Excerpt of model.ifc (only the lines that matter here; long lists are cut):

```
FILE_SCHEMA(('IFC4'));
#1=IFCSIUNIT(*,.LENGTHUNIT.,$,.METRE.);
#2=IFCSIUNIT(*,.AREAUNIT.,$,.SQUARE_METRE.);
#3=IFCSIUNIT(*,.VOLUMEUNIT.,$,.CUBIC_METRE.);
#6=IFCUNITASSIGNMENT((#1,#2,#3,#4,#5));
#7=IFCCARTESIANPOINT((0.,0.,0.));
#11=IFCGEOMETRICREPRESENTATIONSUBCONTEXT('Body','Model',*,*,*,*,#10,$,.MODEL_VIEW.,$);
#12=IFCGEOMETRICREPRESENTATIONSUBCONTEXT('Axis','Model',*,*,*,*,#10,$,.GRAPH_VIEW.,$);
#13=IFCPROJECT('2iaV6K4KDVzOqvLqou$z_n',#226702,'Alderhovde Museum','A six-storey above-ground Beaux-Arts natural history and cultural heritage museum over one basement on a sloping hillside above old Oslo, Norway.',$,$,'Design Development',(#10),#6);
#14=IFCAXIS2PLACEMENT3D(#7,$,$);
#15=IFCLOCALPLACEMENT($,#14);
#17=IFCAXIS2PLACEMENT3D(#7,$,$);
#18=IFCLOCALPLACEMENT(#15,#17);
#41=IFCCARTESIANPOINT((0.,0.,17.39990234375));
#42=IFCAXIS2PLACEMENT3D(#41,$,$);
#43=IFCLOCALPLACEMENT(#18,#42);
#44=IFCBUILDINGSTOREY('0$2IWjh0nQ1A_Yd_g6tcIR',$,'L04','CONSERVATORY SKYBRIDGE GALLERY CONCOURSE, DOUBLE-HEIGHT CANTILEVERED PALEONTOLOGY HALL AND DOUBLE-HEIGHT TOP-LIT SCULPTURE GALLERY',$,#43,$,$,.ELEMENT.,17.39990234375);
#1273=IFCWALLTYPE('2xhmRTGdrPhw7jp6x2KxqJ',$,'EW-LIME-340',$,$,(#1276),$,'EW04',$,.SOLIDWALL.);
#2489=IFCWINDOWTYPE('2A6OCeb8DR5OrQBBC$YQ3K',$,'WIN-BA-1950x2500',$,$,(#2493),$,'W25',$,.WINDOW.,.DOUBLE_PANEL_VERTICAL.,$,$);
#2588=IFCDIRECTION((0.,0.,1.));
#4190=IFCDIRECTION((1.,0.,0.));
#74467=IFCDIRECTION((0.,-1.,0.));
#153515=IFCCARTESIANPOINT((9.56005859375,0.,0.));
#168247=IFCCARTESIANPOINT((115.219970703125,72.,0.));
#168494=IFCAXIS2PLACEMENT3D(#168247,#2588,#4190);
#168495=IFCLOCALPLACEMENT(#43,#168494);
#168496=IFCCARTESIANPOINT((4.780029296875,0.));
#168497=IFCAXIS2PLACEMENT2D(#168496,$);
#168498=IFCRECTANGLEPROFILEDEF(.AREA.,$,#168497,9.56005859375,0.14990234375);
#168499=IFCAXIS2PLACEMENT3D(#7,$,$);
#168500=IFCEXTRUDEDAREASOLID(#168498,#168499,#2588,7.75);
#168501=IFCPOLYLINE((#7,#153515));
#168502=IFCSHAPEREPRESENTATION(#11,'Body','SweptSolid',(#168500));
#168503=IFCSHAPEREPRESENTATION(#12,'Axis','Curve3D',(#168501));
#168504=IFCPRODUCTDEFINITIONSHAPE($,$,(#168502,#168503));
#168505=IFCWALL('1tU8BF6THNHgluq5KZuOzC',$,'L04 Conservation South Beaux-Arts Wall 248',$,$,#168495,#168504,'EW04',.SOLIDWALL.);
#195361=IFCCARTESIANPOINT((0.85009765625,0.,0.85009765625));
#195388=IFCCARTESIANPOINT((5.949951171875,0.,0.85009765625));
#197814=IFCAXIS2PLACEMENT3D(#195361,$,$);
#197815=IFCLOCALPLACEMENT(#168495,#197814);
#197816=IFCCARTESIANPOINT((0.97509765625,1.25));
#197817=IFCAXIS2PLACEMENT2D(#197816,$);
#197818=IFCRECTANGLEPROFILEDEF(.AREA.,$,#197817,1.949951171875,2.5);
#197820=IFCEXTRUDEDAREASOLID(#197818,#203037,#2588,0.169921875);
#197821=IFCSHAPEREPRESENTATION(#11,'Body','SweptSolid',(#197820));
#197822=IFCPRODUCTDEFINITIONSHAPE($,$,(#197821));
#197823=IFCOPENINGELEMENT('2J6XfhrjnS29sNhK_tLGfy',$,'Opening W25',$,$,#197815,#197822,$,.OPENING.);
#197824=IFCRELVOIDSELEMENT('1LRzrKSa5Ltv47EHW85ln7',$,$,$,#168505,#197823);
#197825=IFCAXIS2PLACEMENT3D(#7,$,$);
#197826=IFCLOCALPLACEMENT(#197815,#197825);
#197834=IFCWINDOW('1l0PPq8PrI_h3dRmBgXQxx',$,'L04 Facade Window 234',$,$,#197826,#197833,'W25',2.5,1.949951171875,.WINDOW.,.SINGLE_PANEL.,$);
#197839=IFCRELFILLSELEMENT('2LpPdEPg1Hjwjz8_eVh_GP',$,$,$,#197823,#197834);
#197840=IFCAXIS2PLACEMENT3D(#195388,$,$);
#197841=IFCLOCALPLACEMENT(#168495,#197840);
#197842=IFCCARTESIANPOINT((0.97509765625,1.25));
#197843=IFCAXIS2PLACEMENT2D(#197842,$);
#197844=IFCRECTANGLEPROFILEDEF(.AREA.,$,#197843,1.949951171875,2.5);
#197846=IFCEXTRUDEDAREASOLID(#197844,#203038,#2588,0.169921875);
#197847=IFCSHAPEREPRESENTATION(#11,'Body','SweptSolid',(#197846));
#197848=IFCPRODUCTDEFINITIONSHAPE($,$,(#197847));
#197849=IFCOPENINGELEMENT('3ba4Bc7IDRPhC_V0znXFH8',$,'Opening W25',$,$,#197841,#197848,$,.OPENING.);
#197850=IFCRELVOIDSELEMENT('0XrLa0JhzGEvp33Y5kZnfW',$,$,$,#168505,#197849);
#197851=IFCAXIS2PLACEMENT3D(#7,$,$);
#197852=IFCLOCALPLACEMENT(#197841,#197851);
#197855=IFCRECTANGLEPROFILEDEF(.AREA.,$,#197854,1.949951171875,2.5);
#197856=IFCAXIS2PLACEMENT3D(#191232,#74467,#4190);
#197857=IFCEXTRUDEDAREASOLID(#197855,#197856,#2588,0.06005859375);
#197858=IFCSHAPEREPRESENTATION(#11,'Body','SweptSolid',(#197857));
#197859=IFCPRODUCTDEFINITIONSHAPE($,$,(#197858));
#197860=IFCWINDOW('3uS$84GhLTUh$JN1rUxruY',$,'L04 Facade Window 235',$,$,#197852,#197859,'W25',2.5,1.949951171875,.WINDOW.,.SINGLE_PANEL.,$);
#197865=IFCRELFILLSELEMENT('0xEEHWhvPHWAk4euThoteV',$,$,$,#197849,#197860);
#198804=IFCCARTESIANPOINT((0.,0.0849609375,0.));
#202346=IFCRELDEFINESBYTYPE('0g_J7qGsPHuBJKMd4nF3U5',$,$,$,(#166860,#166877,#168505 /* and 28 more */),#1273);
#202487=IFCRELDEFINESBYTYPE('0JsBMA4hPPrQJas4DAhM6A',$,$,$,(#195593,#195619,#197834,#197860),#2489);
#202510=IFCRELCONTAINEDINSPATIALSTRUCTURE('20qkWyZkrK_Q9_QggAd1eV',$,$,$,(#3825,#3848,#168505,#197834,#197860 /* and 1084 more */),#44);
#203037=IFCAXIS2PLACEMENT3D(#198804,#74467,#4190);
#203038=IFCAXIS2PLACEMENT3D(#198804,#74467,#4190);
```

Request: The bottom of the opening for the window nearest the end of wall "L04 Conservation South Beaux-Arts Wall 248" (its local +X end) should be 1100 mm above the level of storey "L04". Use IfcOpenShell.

```python
import numpy as np
import ifcopenshell
import ifcopenshell.api.geometry
import ifcopenshell.geom
import ifcopenshell.util.element
import ifcopenshell.util.placement
import ifcopenshell.util.shape
import ifcopenshell.util.unit

model = ifcopenshell.open("model.ifc")
unit_scale = ifcopenshell.util.unit.calculate_unit_scale(model)

window = model.by_guid("3uS$84GhLTUh$JN1rUxruY")
opening = window.FillsVoids[0].RelatingOpeningElement
storey = ifcopenshell.util.element.get_container(window, ifc_class="IfcBuildingStorey")
level = ifcopenshell.util.placement.get_local_placement(storey.ObjectPlacement)[2, 3]

# The opening's origin need not be at the sill, so measure its lowest point.
shape = ifcopenshell.geom.create_shape(ifcopenshell.geom.settings(), opening)
bottom = ifcopenshell.util.shape.get_shape_bottom_elevation(shape, shape.geometry) / unit_scale
dz = level + 1.1 - bottom

shift = np.array([0.0, 0.0, dz])
# The window is placed relative to its opening, so it follows when the opening moves.
matrix = ifcopenshell.util.placement.get_local_placement(opening.ObjectPlacement)
matrix[:3, 3] += shift
ifcopenshell.api.geometry.edit_object_placement(
    model, product=opening, matrix=matrix, is_si=False, should_transform_children=True
)

print(f"moved by {dz * unit_scale:+.3f} m")

model.write("model_rev.ifc")
```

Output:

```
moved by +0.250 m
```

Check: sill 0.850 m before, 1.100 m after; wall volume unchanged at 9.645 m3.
